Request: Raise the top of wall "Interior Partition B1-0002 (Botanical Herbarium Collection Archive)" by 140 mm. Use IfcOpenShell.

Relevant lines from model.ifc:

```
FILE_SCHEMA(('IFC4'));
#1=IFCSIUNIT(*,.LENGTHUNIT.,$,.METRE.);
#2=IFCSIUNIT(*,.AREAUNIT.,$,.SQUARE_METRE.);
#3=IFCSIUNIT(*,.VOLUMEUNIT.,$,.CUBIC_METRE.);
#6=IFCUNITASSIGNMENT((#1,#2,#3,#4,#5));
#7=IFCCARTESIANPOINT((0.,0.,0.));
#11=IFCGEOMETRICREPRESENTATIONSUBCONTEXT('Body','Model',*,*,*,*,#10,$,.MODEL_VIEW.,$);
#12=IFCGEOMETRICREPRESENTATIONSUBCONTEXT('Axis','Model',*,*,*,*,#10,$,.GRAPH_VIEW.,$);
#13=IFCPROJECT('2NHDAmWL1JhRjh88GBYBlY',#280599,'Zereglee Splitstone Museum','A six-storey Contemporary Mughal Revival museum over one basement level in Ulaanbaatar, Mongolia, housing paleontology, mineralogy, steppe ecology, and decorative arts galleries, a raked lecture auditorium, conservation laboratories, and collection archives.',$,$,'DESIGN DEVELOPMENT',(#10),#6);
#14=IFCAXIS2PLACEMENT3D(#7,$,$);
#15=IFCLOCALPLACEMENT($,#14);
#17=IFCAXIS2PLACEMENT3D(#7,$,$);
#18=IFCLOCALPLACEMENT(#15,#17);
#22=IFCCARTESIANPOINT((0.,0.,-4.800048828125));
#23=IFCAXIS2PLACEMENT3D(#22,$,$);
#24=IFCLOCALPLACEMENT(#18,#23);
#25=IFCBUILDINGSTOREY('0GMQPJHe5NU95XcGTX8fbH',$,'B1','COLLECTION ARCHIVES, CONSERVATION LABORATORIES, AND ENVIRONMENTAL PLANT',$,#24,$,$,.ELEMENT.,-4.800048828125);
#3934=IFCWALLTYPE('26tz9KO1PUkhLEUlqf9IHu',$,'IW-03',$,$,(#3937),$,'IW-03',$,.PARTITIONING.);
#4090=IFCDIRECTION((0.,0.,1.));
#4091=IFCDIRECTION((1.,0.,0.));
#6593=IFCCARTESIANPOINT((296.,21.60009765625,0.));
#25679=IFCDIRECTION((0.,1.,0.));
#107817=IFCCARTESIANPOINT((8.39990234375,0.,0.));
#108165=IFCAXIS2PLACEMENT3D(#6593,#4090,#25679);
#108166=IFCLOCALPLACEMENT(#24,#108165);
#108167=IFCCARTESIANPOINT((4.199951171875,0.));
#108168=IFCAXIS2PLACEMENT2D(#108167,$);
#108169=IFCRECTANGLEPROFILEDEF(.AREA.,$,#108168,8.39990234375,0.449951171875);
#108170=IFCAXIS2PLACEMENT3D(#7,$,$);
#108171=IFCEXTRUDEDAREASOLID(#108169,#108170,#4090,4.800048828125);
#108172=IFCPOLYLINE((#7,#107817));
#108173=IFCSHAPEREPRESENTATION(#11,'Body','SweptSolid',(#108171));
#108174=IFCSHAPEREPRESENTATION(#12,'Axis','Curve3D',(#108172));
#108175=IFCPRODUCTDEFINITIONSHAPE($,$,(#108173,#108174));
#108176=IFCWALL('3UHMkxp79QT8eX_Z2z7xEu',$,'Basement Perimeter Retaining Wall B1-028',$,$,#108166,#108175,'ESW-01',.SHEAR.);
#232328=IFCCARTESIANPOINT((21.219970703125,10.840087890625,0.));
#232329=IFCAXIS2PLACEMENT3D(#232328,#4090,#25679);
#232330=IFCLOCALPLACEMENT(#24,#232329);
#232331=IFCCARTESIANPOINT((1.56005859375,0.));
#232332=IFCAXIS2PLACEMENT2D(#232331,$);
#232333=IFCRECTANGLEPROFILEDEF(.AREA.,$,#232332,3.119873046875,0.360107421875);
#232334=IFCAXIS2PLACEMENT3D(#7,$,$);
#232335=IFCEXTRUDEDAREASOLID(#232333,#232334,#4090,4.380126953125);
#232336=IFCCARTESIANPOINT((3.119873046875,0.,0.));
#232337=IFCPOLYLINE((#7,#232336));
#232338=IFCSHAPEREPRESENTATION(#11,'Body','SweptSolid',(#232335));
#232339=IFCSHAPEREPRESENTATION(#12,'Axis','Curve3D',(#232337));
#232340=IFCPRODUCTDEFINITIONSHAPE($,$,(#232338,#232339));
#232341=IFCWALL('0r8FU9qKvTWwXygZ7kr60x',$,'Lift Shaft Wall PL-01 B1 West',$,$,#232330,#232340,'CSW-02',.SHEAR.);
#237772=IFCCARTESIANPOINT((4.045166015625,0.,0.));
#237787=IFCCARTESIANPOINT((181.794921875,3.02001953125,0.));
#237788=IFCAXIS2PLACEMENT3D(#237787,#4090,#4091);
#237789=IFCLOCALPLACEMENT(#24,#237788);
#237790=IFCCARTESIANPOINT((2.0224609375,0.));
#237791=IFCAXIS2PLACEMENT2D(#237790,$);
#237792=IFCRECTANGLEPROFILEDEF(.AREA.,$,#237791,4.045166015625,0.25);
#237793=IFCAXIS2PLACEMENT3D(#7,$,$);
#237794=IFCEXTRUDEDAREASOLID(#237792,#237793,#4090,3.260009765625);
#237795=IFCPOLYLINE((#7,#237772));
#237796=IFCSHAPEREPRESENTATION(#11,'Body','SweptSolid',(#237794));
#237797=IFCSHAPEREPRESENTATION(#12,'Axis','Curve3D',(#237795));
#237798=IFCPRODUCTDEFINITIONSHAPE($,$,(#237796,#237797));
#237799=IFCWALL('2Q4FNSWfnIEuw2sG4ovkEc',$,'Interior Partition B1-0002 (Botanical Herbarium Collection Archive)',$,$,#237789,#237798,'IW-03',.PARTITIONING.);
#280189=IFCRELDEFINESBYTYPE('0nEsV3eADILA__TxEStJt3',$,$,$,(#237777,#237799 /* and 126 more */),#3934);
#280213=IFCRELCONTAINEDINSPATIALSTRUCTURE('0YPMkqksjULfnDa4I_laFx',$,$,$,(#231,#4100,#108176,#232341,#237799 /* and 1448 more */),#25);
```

```python
import ifcopenshell
import ifcopenshell.geom
import ifcopenshell.util.representation
import ifcopenshell.util.shape

model = ifcopenshell.open("model.ifc")
settings = ifcopenshell.geom.settings()


def volume(element):
    """Net volume in cubic metres, openings subtracted."""
    shape = ifcopenshell.geom.create_shape(settings, element)
    return ifcopenshell.util.shape.get_volume(shape.geometry)


wall = model.by_id(237799)
before = volume(wall)

body = ifcopenshell.util.representation.get_representation(wall, "Model", "Body")
solid = body.Items[0]
old_height = solid.Depth
solid.Depth += 0.14
after = volume(wall)

print(f"height {old_height:g} -> {solid.Depth:g}, volume {before:.3f} -> {after:.3f} m3")

model.write("model_updated.ifc")
```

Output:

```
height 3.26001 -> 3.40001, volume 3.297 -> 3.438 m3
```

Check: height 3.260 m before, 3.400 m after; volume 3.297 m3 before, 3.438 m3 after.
